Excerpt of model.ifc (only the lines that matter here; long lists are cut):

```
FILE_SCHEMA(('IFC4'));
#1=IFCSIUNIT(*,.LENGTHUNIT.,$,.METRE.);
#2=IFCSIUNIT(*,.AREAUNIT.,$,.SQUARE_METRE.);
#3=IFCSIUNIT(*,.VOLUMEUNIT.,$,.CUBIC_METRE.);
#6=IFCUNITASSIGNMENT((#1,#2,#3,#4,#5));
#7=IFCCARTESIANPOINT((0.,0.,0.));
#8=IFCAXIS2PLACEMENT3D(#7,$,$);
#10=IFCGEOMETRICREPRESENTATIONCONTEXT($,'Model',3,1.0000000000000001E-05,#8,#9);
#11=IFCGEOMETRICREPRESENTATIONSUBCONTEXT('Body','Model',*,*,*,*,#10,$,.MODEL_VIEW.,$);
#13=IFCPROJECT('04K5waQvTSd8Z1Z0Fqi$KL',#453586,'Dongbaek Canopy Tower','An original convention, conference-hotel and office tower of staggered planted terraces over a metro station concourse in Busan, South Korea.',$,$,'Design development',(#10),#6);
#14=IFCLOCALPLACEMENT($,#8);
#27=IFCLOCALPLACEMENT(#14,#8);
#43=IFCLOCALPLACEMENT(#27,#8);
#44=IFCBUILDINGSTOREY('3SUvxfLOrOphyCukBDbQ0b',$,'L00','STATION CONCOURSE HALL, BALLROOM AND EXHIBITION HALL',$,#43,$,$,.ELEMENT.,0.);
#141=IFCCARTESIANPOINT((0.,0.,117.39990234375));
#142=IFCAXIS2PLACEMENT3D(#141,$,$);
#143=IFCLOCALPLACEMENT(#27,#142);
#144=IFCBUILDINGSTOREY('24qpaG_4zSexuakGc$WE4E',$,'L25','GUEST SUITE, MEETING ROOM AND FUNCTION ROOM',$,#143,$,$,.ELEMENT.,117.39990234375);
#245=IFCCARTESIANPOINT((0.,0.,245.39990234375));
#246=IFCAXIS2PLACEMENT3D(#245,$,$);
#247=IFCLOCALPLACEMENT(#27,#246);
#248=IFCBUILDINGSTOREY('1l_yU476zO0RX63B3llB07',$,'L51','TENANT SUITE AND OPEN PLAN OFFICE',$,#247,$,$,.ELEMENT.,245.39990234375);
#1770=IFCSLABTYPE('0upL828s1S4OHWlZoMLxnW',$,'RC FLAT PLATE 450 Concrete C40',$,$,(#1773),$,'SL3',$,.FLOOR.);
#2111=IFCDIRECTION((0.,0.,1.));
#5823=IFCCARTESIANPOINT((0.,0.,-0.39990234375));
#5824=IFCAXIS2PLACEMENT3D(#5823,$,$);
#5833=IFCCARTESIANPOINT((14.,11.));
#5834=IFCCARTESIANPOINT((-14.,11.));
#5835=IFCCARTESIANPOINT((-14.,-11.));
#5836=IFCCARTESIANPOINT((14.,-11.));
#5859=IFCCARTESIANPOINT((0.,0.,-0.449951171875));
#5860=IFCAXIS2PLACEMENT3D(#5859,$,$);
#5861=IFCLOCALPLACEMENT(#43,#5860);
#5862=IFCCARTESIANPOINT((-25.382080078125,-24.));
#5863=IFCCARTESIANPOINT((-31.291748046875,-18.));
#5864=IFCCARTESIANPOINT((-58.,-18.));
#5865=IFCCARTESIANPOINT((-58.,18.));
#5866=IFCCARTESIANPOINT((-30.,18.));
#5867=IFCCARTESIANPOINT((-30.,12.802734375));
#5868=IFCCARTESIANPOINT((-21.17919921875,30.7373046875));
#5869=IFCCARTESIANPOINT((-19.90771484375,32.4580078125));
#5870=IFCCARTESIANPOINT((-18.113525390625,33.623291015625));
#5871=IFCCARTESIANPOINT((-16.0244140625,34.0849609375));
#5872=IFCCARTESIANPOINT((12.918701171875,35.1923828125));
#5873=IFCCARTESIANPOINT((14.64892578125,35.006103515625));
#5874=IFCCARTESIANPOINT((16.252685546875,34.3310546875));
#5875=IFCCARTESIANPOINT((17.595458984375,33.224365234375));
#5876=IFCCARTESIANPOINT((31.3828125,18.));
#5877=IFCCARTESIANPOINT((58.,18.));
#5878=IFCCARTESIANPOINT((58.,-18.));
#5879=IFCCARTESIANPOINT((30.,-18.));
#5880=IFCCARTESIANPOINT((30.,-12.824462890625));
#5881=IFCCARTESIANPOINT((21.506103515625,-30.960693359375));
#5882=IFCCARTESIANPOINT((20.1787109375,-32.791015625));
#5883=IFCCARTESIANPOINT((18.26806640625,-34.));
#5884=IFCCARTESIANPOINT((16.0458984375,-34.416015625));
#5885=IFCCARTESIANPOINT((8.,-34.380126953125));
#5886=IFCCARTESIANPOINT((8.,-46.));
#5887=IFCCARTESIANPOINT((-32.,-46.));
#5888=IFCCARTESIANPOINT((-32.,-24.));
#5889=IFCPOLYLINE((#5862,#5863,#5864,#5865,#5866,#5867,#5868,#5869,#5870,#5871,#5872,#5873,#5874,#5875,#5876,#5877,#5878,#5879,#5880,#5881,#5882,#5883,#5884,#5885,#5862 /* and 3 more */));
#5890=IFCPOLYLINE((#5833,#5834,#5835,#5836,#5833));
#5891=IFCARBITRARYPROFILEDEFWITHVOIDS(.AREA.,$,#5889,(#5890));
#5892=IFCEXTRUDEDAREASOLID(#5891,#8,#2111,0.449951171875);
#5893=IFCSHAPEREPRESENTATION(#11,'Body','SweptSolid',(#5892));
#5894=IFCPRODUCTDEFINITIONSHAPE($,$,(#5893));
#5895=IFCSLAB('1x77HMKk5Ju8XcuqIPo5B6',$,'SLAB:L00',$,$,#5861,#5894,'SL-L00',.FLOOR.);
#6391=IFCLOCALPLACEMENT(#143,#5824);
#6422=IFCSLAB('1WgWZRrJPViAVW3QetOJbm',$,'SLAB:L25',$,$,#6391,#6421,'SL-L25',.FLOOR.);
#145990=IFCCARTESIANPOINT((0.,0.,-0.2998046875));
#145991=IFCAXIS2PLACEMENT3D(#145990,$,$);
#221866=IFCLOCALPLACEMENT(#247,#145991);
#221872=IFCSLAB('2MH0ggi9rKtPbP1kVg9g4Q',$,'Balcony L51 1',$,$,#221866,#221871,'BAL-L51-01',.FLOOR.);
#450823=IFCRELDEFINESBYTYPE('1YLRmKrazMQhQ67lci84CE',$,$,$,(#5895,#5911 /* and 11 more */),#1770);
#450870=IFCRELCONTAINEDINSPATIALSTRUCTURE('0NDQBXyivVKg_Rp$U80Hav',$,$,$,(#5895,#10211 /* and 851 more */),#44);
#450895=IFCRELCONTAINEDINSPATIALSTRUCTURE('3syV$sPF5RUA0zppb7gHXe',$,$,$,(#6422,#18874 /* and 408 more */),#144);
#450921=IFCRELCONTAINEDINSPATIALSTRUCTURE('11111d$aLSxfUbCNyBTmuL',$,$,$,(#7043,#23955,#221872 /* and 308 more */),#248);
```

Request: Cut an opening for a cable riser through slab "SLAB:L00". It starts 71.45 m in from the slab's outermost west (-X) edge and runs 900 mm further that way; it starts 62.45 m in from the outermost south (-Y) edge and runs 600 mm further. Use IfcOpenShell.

```python
import numpy as np
import ifcopenshell
import ifcopenshell.api.feature
import ifcopenshell.api.geometry
import ifcopenshell.api.root
import ifcopenshell.geom
import ifcopenshell.util.placement
import ifcopenshell.util.representation
import ifcopenshell.util.shape
import ifcopenshell.util.unit

model = ifcopenshell.open("model.ifc")
unit_scale = ifcopenshell.util.unit.calculate_unit_scale(model)
settings = ifcopenshell.geom.settings()


def volume(element):
    """Net volume in cubic metres, openings subtracted."""
    shape = ifcopenshell.geom.create_shape(settings, element)
    return ifcopenshell.util.shape.get_volume(shape.geometry)


slab = model.by_guid("1x77HMKk5Ju8XcuqIPo5B6")
before = volume(slab)

# Extent in the slab's own axes, in metres. The edges named are its -X and -Y sides.
slab_shape = ifcopenshell.geom.create_shape(settings, slab)
vertices = ifcopenshell.util.shape.get_vertices(slab_shape.geometry)
x_min, y_min, bottom = vertices.min(axis=0)
top = vertices[:, 2].max()

opening = ifcopenshell.api.root.create_entity(model, ifc_class="IfcOpeningElement", name="Cable riser opening", predefined_type="OPENING")
context = ifcopenshell.util.representation.get_context(model, "Model", "Body", "MODEL_VIEW")
width, depth = 0.9, 0.6
outline = [(0.0, 0.0), (width, 0.0), (width, depth), (0.0, depth), (0.0, 0.0)]
# Overshoot both faces by 50 mm so the cut is clean.
shape = ifcopenshell.api.geometry.add_slab_representation(
    model, context=context, depth=top - bottom + 0.1, polyline=outline
)
ifcopenshell.api.geometry.assign_representation(model, product=opening, representation=shape)

matrix = ifcopenshell.util.placement.get_local_placement(slab.ObjectPlacement)
matrix[:, 3] = matrix @ np.append(np.array([x_min + 71.45, y_min + 62.45, bottom - 0.05]) / unit_scale, 1.0)
ifcopenshell.api.geometry.edit_object_placement(model, product=opening, matrix=matrix, is_si=False)
ifcopenshell.api.feature.add_feature(model, feature=opening, element=slab)

after = volume(slab)

print(f"slab volume {before:.3f} -> {after:.3f} m3")

model.write("model_edited.ifc")
```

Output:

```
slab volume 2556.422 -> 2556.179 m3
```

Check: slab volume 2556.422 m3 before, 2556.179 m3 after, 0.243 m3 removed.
